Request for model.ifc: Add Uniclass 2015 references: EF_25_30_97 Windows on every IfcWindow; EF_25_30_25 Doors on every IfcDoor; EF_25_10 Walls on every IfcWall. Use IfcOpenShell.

First a look at what the model holds.

```python
import ifcopenshell

model = ifcopenshell.open("model.ifc")
print(model.schema)
print("classifications:", [c.Name for c in model.by_type("IfcClassification")])
for ifc_class in ("IfcDoor", "IfcRoof", "IfcStair", "IfcWall", "IfcWindow"):
    print(ifc_class, len(model.by_type(ifc_class)))
```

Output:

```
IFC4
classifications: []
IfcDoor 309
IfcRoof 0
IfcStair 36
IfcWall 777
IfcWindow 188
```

```python
import ifcopenshell
import ifcopenshell.api.classification

model = ifcopenshell.open("model.ifc")

system = ifcopenshell.api.classification.add_classification(model, classification="Uniclass 2015")

codes = {
    "IfcWindow": ("EF_25_30_97", "Windows"),
    "IfcDoor": ("EF_25_30_25", "Doors"),
    "IfcWall": ("EF_25_10", "Walls"),
}
for ifc_class, (code, name) in codes.items():
    products = model.by_type(ifc_class)
    ifcopenshell.api.classification.add_reference(
        model, products=products, classification=system, identification=code, name=name
    )
    print(code, len(products))

model.write("model_edited.ifc")
```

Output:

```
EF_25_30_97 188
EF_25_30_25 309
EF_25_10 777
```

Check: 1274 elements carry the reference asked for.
